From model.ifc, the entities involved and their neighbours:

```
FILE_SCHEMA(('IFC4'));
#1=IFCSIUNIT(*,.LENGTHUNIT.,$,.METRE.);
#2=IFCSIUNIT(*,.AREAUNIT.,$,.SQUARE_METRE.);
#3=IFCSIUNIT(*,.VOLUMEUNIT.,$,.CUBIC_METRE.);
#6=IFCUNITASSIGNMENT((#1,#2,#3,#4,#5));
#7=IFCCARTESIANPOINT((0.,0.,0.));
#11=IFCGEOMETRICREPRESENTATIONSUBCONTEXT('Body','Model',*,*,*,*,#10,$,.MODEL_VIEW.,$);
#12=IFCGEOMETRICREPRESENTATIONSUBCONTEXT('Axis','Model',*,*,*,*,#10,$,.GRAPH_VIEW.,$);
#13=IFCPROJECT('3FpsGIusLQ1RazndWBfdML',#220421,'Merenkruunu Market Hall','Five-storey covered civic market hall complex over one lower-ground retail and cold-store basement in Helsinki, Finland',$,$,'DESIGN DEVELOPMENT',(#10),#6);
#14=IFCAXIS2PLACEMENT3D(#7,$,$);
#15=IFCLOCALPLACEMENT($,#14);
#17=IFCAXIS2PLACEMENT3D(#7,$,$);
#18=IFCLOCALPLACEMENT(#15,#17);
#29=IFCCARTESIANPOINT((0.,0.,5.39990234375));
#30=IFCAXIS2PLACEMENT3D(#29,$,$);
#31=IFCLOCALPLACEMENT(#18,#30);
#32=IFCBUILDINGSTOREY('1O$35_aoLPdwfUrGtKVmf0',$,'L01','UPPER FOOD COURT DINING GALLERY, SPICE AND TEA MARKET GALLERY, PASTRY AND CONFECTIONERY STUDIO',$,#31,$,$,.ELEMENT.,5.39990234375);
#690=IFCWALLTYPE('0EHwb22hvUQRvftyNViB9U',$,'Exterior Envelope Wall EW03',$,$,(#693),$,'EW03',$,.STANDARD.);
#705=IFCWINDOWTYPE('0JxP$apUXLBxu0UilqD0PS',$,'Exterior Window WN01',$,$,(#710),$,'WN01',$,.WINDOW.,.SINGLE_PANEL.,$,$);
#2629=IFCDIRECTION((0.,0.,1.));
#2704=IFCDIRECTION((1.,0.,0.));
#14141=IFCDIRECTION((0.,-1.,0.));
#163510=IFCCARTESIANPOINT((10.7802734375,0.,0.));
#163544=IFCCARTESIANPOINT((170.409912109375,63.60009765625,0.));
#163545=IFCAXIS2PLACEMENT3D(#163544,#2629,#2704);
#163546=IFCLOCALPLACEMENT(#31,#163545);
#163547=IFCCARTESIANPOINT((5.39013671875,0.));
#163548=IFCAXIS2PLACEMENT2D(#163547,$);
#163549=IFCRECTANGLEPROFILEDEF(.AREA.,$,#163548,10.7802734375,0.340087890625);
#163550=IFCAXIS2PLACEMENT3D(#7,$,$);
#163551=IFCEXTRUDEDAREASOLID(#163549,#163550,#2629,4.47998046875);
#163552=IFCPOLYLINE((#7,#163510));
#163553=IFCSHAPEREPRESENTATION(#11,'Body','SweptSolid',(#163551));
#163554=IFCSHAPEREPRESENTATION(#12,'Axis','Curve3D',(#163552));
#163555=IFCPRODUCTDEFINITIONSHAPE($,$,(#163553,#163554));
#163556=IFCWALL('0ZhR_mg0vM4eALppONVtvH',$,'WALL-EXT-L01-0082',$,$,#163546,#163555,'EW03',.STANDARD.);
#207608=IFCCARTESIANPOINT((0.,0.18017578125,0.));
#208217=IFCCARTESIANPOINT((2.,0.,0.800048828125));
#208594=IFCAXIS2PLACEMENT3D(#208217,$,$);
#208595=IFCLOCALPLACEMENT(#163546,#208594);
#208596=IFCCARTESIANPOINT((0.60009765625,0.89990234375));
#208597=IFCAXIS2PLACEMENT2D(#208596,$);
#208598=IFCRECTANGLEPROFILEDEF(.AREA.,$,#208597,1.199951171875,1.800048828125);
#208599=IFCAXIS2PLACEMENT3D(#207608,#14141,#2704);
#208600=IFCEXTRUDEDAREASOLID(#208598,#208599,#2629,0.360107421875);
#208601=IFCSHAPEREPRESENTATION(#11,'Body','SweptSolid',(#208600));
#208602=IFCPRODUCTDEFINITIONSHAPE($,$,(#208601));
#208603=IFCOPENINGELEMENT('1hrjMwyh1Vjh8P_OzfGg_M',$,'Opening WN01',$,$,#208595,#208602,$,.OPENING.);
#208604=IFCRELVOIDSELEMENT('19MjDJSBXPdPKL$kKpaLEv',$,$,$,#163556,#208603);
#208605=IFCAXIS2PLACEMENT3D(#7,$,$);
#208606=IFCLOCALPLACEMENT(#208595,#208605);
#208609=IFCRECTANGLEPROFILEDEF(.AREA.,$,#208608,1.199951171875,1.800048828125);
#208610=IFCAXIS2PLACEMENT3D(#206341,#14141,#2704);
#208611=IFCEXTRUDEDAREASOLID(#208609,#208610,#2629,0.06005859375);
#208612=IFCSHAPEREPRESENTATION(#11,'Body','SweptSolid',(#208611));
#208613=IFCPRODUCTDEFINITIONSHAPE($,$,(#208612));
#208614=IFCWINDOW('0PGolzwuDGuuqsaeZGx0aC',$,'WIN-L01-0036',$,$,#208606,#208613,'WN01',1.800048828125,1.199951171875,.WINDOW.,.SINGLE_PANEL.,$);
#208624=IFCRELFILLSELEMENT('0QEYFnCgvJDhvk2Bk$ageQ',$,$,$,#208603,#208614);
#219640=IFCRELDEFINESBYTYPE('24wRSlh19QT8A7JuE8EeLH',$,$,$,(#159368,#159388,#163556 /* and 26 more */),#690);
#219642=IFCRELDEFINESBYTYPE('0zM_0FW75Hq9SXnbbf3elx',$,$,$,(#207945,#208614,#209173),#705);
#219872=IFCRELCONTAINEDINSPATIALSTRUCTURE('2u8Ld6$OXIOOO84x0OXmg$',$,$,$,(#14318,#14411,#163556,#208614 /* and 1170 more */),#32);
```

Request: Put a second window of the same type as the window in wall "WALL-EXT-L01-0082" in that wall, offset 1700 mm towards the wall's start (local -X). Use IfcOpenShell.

```python
import ifcopenshell
import ifcopenshell.api.feature
import ifcopenshell.api.geometry
import ifcopenshell.api.root
import ifcopenshell.geom
import ifcopenshell.util.element
import ifcopenshell.util.placement
import ifcopenshell.util.shape

model = ifcopenshell.open("model.ifc")
settings = ifcopenshell.geom.settings()


def volume(element):
    """Net volume in cubic metres, openings subtracted."""
    shape = ifcopenshell.geom.create_shape(settings, element)
    return ifcopenshell.util.shape.get_volume(shape.geometry)


window = model.by_guid("0PGolzwuDGuuqsaeZGx0aC")
opening = window.FillsVoids[0].RelatingOpeningElement
wall = opening.VoidsElements[0].RelatingBuildingElement
before = volume(wall)
shift = ifcopenshell.util.placement.get_local_placement(wall.ObjectPlacement)[:3, 0] * -1.7

# copy_class copies the void relationship, type, container and properties, but no geometry.
new_opening = ifcopenshell.api.root.copy_class(model, product=opening)
new_opening.Representation = ifcopenshell.util.element.copy_deep(
    model, opening.Representation, exclude=["IfcGeometricRepresentationContext", "IfcRepresentationMap"]
)
new_window = ifcopenshell.api.root.copy_class(model, product=window)
new_window.Representation = ifcopenshell.util.element.copy_deep(
    model, window.Representation, exclude=["IfcGeometricRepresentationContext", "IfcRepresentationMap"]
)
new_window.Tag = None
ifcopenshell.api.feature.add_filling(model, opening=new_opening, element=new_window)

for old, new in ((opening, new_opening), (window, new_window)):
    matrix = ifcopenshell.util.placement.get_local_placement(old.ObjectPlacement)
    matrix[:3, 3] += shift
    ifcopenshell.api.geometry.edit_object_placement(model, product=new, matrix=matrix, is_si=False)

after = volume(wall)

print(f"wall volume {before:.3f} -> {after:.3f} m3")

model.write("model-out.ifc")
```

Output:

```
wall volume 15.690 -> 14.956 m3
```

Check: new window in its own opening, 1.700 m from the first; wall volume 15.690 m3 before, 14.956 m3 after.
